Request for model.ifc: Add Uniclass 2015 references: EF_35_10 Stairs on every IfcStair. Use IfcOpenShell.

First a look at what the model holds.

```python
import ifcopenshell

model = ifcopenshell.open("model.ifc")
print(model.schema)
print("classifications:", [c.Name for c in model.by_type("IfcClassification")])
for ifc_class in ("IfcDoor", "IfcRoof", "IfcStair", "IfcWall", "IfcWindow"):
    print(ifc_class, len(model.by_type(ifc_class)))
```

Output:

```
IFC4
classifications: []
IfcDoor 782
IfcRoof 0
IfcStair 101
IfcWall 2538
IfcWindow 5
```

```python
import ifcopenshell
import ifcopenshell.api.classification

model = ifcopenshell.open("model.ifc")

system = ifcopenshell.api.classification.add_classification(model, classification="Uniclass 2015")

codes = {
    "IfcStair": ("EF_35_10", "Stairs"),
}
for ifc_class, (code, name) in codes.items():
    products = model.by_type(ifc_class)
    ifcopenshell.api.classification.add_reference(
        model, products=products, classification=system, identification=code, name=name
    )
    print(code, len(products))

model.write("model_edited.ifc")
```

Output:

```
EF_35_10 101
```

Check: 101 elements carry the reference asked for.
